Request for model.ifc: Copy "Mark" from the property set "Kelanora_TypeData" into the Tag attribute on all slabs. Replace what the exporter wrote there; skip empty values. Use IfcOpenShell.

First a look at what the model holds.

```python
import ifcopenshell
import ifcopenshell.util.element

model = ifcopenshell.open("model.ifc")
print(model.schema)
slabs = model.by_type("IfcSlab")
print(len(slabs), "slabs")
for e in slabs[:8]:
    source = ifcopenshell.util.element.get_pset(e, "Kelanora_TypeData", "Mark")
    target = e.Tag
    print(e.id(), repr(source), repr(target), sep=" | ")
```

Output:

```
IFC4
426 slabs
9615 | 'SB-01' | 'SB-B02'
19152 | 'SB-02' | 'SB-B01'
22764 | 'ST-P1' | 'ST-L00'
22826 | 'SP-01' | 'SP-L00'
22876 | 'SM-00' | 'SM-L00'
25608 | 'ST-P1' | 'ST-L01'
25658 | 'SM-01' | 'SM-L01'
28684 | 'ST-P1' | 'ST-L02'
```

```python
import ifcopenshell
import ifcopenshell.util.element

model = ifcopenshell.open("model.ifc")

count = 0
for e in model.by_type("IfcSlab"):
    value = ifcopenshell.util.element.get_pset(e, "Kelanora_TypeData", "Mark")
    current = e.Tag
    if not value or not value.strip() or current == value:
        continue
    e.Tag = value
    count += 1

print(count, "slabs updated")

model.write("model_updated.ifc")
```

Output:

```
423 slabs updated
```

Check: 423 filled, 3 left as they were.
